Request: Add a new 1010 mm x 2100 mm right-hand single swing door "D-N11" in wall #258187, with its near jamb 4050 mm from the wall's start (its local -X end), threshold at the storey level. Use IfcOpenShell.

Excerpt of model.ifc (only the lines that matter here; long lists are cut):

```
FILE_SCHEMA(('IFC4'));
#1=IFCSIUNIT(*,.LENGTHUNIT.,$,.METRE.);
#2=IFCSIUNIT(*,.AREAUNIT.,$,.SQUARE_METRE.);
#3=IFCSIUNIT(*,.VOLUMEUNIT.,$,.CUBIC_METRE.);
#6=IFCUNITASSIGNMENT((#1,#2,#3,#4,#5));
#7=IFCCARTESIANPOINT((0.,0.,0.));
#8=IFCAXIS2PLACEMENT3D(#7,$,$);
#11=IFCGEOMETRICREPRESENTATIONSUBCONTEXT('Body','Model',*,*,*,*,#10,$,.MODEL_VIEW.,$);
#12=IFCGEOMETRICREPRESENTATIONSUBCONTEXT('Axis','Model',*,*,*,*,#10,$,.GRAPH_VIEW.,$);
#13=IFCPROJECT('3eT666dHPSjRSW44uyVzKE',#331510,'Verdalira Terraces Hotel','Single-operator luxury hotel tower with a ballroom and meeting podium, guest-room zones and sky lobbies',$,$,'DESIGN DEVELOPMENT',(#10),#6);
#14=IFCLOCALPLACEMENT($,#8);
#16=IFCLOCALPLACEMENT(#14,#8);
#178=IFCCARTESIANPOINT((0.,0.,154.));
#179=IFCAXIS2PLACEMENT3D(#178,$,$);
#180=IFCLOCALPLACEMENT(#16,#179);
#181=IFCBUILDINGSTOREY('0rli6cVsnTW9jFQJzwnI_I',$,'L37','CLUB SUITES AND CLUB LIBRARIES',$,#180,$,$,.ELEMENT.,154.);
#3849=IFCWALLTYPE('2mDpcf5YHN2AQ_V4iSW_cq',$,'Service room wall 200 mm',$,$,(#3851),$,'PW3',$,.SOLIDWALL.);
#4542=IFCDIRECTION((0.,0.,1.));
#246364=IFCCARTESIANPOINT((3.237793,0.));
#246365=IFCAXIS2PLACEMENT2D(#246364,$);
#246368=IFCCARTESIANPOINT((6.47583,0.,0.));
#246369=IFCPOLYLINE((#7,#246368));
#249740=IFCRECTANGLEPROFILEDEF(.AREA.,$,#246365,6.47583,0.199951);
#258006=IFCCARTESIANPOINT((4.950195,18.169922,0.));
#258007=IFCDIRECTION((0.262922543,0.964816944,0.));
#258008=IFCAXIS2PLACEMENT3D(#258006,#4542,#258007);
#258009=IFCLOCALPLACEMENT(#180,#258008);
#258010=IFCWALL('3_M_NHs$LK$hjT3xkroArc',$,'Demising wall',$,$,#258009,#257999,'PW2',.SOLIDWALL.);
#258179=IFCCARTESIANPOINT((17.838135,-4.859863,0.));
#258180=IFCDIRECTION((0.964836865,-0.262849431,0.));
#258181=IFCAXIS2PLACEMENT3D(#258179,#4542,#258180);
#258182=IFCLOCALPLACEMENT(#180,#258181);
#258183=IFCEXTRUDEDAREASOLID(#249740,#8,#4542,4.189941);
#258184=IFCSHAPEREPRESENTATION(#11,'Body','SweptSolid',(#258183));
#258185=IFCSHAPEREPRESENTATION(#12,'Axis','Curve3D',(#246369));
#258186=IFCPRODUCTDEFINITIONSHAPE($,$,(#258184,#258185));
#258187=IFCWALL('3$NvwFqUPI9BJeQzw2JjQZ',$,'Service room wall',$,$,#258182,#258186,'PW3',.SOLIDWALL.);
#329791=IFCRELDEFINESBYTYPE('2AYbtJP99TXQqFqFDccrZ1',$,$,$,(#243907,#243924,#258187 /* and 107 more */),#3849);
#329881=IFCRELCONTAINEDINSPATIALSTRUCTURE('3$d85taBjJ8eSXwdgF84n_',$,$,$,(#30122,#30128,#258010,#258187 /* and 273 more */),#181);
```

```python
import numpy as np
import ifcopenshell
import ifcopenshell.api.feature
import ifcopenshell.api.geometry
import ifcopenshell.api.root
import ifcopenshell.api.spatial
import ifcopenshell.geom
import ifcopenshell.util.element
import ifcopenshell.util.placement
import ifcopenshell.util.representation
import ifcopenshell.util.shape
import ifcopenshell.util.unit

model = ifcopenshell.open("model.ifc")
unit_scale = ifcopenshell.util.unit.calculate_unit_scale(model)
settings = ifcopenshell.geom.settings()


def volume(element):
    """Net volume in cubic metres, openings subtracted."""
    shape = ifcopenshell.geom.create_shape(settings, element)
    return ifcopenshell.util.shape.get_volume(shape.geometry)


wall = model.by_guid("3$NvwFqUPI9BJeQzw2JjQZ")
storey = ifcopenshell.util.element.get_container(wall, ifc_class="IfcBuildingStorey")
context = ifcopenshell.util.representation.get_context(model, "Model", "Body", "MODEL_VIEW")
before = volume(wall)

width, height, from_end, sill = 1.01, 2.1, 4.05, 0.0  # metres

# The wall runs along its own X axis, and the end named is its -X end.
wall_shape = ifcopenshell.geom.create_shape(settings, wall)
x, y, z = ifcopenshell.util.shape.get_vertices(wall_shape.geometry).T
start = x.min() + from_end
face, thickness = float(y.min()), float(y.max() - y.min())
wall_matrix = ifcopenshell.util.placement.get_local_placement(wall.ObjectPlacement)
level = ifcopenshell.util.placement.get_local_placement(storey.ObjectPlacement)[2, 3]


def in_wall(x, y):
    """Placement at x, y metres in the wall's axes, at sill height."""
    matrix = wall_matrix.copy()
    matrix[:, 3] = wall_matrix @ np.array([x / unit_scale, y / unit_scale, 0.0, 1.0])
    matrix[2, 3] = level + sill / unit_scale
    return matrix


# Opening: a box that overshoots both wall faces by 50 mm.
opening = ifcopenshell.api.root.create_entity(model, ifc_class="IfcOpeningElement", predefined_type="OPENING")
box = ifcopenshell.api.geometry.add_wall_representation(
    model, context=context, length=width, height=height, thickness=thickness + 0.1
)
ifcopenshell.api.geometry.assign_representation(model, product=opening, representation=box)
ifcopenshell.api.geometry.edit_object_placement(model, product=opening, matrix=in_wall(start, face - 0.05), is_si=False)
ifcopenshell.api.feature.add_feature(model, feature=opening, element=wall)

door = ifcopenshell.api.root.create_entity(model, ifc_class="IfcDoor", name="D-N11", predefined_type="DOOR")
door.OverallWidth, door.OverallHeight = width / unit_scale, height / unit_scale
door.OperationType = "SINGLE_SWING_RIGHT"
body = ifcopenshell.api.geometry.add_door_representation(
    model,
    context=context,
    overall_width=door.OverallWidth,
    overall_height=door.OverallHeight,
    operation_type="SINGLE_SWING_RIGHT",
    lining_properties={"LiningDepth": thickness / unit_scale, "ThresholdDepth": thickness / unit_scale},
)
ifcopenshell.api.geometry.assign_representation(model, product=door, representation=body)
ifcopenshell.api.spatial.assign_container(model, products=[door], relating_structure=storey)
ifcopenshell.api.feature.add_filling(model, opening=opening, element=door)

# The lining spans the wall, so the door starts at the wall face.
ifcopenshell.api.geometry.edit_object_placement(model, product=door, matrix=in_wall(start, face), is_si=False)

after = volume(wall)

print(f"wall volume {before:.3f} -> {after:.3f} m3")

model.write("model_edited.ifc")
```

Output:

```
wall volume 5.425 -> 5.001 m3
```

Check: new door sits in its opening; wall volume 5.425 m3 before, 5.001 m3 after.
